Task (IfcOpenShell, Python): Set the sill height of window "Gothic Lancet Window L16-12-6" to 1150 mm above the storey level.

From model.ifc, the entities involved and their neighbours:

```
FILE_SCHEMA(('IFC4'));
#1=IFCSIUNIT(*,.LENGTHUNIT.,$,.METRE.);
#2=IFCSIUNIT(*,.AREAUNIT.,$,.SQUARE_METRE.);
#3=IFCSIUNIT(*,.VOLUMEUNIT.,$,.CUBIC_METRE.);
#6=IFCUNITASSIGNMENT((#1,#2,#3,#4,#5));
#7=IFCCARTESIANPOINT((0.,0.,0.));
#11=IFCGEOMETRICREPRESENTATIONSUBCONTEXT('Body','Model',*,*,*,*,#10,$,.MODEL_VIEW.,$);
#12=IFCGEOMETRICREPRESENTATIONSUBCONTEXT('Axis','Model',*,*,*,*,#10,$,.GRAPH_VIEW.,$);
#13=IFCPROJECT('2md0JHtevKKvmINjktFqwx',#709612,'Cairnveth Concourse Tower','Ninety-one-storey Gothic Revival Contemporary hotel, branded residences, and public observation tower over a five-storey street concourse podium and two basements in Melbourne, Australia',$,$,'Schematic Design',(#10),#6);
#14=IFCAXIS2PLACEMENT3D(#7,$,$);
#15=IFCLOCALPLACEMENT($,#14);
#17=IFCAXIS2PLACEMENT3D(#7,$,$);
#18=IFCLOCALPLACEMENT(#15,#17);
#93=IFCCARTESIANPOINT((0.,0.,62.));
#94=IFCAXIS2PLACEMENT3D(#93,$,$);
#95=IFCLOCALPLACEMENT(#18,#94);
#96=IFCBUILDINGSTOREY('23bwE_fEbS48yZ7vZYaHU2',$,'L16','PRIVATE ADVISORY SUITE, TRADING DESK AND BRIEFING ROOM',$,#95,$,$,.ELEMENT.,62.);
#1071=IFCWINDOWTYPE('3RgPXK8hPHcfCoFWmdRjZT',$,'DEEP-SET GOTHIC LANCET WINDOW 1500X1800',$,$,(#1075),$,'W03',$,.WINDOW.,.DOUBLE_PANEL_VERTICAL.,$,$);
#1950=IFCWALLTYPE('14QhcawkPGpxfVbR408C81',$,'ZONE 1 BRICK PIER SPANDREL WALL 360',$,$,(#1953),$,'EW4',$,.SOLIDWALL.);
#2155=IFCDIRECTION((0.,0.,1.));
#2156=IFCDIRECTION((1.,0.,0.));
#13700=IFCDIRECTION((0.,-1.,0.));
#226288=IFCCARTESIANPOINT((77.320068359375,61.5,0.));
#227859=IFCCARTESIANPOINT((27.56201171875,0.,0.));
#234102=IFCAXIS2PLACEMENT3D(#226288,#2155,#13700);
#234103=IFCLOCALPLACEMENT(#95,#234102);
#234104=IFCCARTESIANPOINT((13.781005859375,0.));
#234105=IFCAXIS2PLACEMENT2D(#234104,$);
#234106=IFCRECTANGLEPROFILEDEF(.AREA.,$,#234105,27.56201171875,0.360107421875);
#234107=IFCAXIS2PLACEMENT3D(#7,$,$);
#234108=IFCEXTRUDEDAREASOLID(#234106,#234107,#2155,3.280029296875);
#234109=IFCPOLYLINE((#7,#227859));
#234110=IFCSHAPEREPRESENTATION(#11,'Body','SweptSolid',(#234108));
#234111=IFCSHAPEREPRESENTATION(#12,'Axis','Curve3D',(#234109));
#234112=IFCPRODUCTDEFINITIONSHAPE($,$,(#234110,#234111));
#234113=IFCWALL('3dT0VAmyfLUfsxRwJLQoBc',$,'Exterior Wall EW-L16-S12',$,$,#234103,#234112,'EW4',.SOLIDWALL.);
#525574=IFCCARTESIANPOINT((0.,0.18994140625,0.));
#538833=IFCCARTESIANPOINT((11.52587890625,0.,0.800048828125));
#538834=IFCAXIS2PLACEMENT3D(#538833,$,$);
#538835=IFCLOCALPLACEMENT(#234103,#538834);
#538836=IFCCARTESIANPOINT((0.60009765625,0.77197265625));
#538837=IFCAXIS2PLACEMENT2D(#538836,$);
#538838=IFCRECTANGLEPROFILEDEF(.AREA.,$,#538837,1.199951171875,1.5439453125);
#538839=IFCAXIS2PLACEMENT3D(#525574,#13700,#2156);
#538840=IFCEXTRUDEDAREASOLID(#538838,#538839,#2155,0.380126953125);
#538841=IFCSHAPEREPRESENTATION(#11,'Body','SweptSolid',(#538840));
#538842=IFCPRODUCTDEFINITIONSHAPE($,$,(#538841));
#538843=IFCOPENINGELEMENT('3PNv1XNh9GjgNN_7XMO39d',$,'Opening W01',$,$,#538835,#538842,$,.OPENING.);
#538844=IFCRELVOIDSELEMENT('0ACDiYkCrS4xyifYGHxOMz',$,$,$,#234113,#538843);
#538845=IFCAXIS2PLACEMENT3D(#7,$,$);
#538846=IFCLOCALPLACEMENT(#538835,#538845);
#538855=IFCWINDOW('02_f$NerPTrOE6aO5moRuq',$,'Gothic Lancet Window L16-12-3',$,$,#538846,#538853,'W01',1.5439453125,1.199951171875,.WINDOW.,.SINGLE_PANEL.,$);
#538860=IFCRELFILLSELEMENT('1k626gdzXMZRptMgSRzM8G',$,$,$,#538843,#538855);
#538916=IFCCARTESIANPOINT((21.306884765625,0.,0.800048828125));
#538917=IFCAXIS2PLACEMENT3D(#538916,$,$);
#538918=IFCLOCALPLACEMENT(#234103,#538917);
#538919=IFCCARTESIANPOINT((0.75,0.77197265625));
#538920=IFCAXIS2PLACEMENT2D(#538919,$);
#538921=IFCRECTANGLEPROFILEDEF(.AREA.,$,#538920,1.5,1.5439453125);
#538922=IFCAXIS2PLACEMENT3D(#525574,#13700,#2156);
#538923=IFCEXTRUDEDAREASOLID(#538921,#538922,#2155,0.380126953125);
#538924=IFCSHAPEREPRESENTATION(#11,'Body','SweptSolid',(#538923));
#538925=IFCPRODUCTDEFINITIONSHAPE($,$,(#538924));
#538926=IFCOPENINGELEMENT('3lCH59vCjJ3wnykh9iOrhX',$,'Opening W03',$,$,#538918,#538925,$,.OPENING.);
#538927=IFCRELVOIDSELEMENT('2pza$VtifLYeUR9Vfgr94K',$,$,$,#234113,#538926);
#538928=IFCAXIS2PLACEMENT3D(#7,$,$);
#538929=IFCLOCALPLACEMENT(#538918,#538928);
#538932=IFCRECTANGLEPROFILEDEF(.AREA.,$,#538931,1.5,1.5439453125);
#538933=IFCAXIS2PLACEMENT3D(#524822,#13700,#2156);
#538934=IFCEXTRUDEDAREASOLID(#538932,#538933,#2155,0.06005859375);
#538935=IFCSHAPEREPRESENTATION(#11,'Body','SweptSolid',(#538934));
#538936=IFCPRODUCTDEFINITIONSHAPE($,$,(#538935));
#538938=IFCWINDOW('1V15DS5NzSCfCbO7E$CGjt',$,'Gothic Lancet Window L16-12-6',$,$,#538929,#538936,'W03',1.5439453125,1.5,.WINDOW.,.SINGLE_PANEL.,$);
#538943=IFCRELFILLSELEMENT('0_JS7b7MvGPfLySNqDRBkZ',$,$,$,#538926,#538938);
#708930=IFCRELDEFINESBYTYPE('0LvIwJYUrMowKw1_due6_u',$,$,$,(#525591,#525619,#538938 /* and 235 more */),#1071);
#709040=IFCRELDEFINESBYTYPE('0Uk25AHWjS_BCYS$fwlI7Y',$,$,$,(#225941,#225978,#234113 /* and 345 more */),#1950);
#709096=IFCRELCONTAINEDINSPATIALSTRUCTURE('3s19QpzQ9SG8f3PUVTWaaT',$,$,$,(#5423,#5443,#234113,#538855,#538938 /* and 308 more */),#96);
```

```python
import numpy as np
import ifcopenshell
import ifcopenshell.api.geometry
import ifcopenshell.geom
import ifcopenshell.util.element
import ifcopenshell.util.placement
import ifcopenshell.util.shape
import ifcopenshell.util.unit

model = ifcopenshell.open("model.ifc")
unit_scale = ifcopenshell.util.unit.calculate_unit_scale(model)

window = model.by_id(538938)
opening = window.FillsVoids[0].RelatingOpeningElement
storey = ifcopenshell.util.element.get_container(window, ifc_class="IfcBuildingStorey")
level = ifcopenshell.util.placement.get_local_placement(storey.ObjectPlacement)[2, 3]

# The opening's origin need not be at the sill, so measure its lowest point.
shape = ifcopenshell.geom.create_shape(ifcopenshell.geom.settings(), opening)
bottom = ifcopenshell.util.shape.get_shape_bottom_elevation(shape, shape.geometry) / unit_scale
dz = level + 1.15 / unit_scale - bottom

shift = np.array([0.0, 0.0, dz])
# The window is placed relative to its opening, so it follows when the opening moves.
matrix = ifcopenshell.util.placement.get_local_placement(opening.ObjectPlacement)
matrix[:3, 3] += shift
ifcopenshell.api.geometry.edit_object_placement(
    model, product=opening, matrix=matrix, is_si=False, should_transform_children=True
)

print(f"moved by {dz * unit_scale:+.3f} m")

model.write("model_rev.ifc")
```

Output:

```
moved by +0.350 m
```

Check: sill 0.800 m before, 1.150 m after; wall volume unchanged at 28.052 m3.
